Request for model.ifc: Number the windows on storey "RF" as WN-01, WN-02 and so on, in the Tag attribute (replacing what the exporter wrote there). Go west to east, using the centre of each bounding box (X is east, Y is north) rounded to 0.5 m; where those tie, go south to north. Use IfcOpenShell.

First a look at what the model holds.

```python
import ifcopenshell
import ifcopenshell.util.element
import ifcopenshell.util.placement

model = ifcopenshell.open("model.ifc")
print(model.schema)
storey = next(s for s in model.by_type("IfcBuildingStorey") if s.Name == "RF")
windows = [e for e in ifcopenshell.util.element.get_decomposition(storey) if e.is_a("IfcWindow")]
for e in sorted(windows, key=lambda e: e.id()):
    origin = ifcopenshell.util.placement.get_local_placement(e.ObjectPlacement)[:3, 3]
    print(e.id(), e.Tag, e.Name, origin.round(2) + 0.0, sep=" | ")
```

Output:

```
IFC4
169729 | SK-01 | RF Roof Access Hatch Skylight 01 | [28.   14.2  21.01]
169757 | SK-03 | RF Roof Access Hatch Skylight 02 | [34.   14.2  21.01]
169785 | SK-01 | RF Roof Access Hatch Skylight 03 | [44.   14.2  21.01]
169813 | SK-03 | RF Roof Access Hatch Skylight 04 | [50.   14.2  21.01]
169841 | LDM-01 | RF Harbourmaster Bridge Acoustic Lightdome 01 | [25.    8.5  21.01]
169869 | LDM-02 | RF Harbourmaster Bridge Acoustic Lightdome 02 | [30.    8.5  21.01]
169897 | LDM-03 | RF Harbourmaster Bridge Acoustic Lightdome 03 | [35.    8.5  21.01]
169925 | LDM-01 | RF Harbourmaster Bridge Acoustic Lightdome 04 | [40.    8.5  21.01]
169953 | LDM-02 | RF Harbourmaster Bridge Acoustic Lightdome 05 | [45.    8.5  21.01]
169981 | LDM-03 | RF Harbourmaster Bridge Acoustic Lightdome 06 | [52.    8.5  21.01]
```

```python
import ifcopenshell
import ifcopenshell.geom
import ifcopenshell.util.element
import ifcopenshell.util.shape

model = ifcopenshell.open("model.ifc")
settings = ifcopenshell.geom.settings()
settings.set("use-world-coords", True)


def centre(element):
    shape = ifcopenshell.geom.create_shape(settings, element)
    return ifcopenshell.util.shape.get_bbox_centroid(shape.geometry)


storey = next(s for s in model.by_type("IfcBuildingStorey") if s.Name == "RF")
windows = [e for e in ifcopenshell.util.element.get_decomposition(storey) if e.is_a("IfcWindow")]

# Insertion points can sit at a corner or the storey origin, so sort by the geometry (in metres).
centres = {e: centre(e) for e in windows}
windows.sort(key=lambda e: (round(centres[e][0] / 0.5), centres[e][1]))

for i, e in enumerate(windows, start=1):
    number = f"WN-{i:02d}"
    e.Tag = number
    print(e.id(), number)

model.write("model_v2.ifc")
```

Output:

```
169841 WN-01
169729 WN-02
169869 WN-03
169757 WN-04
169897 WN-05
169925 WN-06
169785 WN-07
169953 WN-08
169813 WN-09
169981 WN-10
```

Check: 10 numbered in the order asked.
